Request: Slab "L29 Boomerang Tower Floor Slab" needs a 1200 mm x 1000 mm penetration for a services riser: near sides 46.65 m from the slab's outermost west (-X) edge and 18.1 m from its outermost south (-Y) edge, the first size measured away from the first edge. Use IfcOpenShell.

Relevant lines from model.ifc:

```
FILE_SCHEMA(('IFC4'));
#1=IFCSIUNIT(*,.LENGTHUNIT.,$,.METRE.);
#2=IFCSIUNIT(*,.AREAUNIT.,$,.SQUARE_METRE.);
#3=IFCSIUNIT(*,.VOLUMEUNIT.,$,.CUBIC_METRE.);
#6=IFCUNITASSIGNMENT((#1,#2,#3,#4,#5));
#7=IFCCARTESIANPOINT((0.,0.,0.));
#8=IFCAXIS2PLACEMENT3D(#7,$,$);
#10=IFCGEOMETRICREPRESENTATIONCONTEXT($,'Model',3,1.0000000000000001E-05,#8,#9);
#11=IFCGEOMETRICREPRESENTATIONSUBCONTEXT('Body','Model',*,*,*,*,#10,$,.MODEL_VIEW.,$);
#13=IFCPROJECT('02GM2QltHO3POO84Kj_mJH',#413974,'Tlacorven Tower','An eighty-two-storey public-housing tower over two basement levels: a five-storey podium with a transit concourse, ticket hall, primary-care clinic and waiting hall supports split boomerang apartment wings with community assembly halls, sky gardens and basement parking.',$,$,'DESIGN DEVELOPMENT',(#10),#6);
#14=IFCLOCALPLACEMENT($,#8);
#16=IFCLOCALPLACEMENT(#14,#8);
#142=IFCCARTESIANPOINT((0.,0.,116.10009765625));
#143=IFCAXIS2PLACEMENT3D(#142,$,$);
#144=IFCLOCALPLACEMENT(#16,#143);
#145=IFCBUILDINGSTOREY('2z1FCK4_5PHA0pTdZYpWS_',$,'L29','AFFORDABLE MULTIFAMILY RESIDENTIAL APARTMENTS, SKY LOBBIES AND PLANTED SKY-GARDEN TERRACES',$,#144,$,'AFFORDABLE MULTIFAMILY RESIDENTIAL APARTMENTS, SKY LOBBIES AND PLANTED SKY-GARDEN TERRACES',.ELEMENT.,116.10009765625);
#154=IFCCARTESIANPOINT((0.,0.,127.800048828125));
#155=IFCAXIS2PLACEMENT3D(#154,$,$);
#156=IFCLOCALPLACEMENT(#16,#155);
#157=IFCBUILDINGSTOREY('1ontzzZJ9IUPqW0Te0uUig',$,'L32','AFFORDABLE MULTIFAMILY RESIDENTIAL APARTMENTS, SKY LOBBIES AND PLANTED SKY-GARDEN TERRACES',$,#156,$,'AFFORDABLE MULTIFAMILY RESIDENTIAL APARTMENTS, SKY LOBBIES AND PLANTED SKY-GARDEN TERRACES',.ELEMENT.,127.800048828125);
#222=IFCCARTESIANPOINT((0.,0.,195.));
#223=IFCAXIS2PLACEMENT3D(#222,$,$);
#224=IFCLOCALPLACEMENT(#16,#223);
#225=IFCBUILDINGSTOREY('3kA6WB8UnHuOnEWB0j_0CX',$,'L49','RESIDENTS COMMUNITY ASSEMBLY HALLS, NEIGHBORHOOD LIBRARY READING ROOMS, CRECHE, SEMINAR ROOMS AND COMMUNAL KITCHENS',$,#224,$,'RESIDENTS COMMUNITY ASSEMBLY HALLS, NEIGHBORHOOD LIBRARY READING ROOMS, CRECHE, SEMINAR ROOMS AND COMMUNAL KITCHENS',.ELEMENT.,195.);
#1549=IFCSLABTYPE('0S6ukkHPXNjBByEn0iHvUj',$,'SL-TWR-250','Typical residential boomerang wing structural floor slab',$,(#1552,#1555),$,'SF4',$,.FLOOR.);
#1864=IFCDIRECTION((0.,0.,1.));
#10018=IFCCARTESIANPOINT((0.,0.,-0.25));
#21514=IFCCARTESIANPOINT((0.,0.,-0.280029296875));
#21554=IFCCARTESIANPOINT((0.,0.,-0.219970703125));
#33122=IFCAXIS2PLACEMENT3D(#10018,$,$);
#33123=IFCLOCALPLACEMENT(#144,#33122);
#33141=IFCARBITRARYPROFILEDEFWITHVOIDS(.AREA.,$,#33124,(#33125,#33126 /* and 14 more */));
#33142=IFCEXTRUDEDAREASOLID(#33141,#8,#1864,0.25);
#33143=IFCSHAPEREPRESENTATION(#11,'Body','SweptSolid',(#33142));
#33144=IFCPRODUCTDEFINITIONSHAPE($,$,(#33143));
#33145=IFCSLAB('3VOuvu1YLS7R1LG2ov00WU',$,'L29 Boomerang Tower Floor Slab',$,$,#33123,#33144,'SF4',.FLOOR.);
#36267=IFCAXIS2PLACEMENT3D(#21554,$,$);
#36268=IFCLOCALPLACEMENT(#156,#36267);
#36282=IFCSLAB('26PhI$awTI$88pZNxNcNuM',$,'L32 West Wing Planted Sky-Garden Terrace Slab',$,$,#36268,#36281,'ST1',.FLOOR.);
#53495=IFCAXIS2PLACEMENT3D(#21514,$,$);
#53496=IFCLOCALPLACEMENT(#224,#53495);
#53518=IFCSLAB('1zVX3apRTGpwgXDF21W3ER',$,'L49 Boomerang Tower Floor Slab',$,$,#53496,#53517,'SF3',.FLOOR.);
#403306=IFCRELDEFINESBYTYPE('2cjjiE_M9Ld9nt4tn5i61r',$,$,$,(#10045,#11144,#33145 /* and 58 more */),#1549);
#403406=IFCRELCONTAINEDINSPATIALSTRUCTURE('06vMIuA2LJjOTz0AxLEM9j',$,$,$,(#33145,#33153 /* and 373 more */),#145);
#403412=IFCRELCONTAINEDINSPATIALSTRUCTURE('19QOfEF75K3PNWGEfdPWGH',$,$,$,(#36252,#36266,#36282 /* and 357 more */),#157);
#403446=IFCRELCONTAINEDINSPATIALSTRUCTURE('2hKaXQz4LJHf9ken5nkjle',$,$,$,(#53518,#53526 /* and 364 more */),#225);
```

```python
import numpy as np
import ifcopenshell
import ifcopenshell.api.feature
import ifcopenshell.api.geometry
import ifcopenshell.api.root
import ifcopenshell.geom
import ifcopenshell.util.placement
import ifcopenshell.util.representation
import ifcopenshell.util.shape
import ifcopenshell.util.unit

model = ifcopenshell.open("model.ifc")
unit_scale = ifcopenshell.util.unit.calculate_unit_scale(model)
settings = ifcopenshell.geom.settings()


def volume(element):
    """Net volume in cubic metres, openings subtracted."""
    shape = ifcopenshell.geom.create_shape(settings, element)
    return ifcopenshell.util.shape.get_volume(shape.geometry)


slab = model.by_guid("3VOuvu1YLS7R1LG2ov00WU")
before = volume(slab)

# Extent in the slab's own axes, in metres. The edges named are its -X and -Y sides.
slab_shape = ifcopenshell.geom.create_shape(settings, slab)
vertices = ifcopenshell.util.shape.get_vertices(slab_shape.geometry)
x_min, y_min, bottom = vertices.min(axis=0)
top = vertices[:, 2].max()

opening = ifcopenshell.api.root.create_entity(model, ifc_class="IfcOpeningElement", name="Services riser opening", predefined_type="OPENING")
context = ifcopenshell.util.representation.get_context(model, "Model", "Body", "MODEL_VIEW")
width, depth = 1.2, 1
outline = [(0.0, 0.0), (width, 0.0), (width, depth), (0.0, depth), (0.0, 0.0)]
# Overshoot both faces by 50 mm so the cut is clean.
shape = ifcopenshell.api.geometry.add_slab_representation(
    model, context=context, depth=top - bottom + 0.1, polyline=outline
)
ifcopenshell.api.geometry.assign_representation(model, product=opening, representation=shape)

matrix = ifcopenshell.util.placement.get_local_placement(slab.ObjectPlacement)
matrix[:, 3] = matrix @ np.append(np.array([x_min + 46.65, y_min + 18.1, bottom - 0.05]) / unit_scale, 1.0)
ifcopenshell.api.geometry.edit_object_placement(model, product=opening, matrix=matrix, is_si=False)
ifcopenshell.api.feature.add_feature(model, feature=opening, element=slab)

after = volume(slab)

print(f"slab volume {before:.3f} -> {after:.3f} m3")

model.write("model-out.ifc")
```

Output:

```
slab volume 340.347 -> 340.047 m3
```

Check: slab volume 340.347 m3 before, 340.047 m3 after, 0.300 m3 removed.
